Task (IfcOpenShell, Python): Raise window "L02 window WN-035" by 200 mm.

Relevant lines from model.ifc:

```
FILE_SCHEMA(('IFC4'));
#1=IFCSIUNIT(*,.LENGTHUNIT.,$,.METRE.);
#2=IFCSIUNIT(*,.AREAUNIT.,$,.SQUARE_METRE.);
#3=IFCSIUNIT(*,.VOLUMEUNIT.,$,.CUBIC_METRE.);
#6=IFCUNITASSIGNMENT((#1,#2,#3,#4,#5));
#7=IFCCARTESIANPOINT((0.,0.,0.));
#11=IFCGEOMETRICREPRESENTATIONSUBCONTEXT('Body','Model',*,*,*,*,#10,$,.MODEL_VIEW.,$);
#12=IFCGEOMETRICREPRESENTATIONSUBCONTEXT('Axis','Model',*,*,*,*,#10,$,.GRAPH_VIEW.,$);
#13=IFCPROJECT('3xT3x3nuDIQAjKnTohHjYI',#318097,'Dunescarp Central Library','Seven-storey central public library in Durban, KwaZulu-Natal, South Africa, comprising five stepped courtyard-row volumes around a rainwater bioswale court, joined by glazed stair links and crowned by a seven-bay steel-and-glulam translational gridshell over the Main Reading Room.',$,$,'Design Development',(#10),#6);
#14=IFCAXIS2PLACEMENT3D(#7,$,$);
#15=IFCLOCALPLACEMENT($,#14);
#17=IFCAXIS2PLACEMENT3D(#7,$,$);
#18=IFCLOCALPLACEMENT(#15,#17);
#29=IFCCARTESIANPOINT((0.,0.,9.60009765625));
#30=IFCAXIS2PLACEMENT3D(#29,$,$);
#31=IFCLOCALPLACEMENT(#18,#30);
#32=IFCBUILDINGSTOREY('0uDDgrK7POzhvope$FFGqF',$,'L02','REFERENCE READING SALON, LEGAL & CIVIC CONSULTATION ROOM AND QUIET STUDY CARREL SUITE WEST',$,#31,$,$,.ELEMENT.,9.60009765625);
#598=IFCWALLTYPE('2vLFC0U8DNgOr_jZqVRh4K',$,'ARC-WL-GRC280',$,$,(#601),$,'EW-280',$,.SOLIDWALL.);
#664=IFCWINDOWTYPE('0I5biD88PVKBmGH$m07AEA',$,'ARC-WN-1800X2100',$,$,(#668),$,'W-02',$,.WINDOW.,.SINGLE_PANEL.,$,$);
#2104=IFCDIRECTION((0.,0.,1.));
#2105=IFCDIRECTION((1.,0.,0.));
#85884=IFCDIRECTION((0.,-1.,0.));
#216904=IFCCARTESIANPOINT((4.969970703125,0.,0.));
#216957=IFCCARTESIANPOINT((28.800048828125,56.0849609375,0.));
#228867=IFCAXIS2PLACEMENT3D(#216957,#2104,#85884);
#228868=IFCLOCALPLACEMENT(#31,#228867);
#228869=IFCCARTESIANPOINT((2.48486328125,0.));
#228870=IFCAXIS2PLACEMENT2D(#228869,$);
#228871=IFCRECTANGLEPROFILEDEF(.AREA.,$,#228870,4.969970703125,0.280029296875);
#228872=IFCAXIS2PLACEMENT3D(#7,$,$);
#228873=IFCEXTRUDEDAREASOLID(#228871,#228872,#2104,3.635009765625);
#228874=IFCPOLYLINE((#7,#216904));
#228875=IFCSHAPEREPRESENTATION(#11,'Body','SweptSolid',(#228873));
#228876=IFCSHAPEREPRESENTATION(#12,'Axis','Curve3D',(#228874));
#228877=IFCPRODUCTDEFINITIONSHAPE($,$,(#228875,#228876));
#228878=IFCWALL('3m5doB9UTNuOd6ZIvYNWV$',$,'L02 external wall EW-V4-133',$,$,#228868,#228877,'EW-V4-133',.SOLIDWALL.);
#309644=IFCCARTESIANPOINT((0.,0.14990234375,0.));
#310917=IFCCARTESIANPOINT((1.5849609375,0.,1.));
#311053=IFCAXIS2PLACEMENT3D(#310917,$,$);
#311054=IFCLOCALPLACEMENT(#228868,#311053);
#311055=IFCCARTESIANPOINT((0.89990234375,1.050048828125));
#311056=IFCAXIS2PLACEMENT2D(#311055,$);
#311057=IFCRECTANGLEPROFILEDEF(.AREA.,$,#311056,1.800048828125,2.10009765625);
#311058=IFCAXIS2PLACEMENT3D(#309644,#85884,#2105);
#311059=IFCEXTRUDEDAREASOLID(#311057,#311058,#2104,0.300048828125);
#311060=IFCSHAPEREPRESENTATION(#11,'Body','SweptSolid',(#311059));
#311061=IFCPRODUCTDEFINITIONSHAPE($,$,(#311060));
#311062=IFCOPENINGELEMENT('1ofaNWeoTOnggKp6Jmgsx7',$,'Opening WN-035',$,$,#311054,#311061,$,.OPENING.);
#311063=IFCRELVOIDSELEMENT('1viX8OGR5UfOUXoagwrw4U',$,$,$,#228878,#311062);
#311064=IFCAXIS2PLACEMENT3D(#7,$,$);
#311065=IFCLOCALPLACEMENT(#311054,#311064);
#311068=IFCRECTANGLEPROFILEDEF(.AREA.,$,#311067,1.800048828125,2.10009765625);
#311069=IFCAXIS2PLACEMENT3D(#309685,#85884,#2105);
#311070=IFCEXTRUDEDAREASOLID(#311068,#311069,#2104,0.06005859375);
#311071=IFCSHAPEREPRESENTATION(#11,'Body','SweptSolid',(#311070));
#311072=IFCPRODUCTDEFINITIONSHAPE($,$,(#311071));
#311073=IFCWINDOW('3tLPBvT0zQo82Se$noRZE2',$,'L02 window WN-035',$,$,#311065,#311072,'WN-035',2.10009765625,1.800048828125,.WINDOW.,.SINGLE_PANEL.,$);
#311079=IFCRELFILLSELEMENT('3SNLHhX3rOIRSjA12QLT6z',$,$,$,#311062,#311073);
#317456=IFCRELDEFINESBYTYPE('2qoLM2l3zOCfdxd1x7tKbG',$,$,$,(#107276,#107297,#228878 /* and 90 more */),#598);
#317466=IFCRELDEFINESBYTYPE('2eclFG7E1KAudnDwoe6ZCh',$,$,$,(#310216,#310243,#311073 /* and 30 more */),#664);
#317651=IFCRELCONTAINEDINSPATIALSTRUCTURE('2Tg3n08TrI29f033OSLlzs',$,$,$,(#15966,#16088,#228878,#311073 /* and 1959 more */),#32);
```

```python
import numpy as np
import ifcopenshell
import ifcopenshell.api.geometry
import ifcopenshell.util.placement
import ifcopenshell.util.unit

model = ifcopenshell.open("model.ifc")
unit_scale = ifcopenshell.util.unit.calculate_unit_scale(model)

window = model.by_guid("3tLPBvT0zQo82Se$noRZE2")
opening = window.FillsVoids[0].RelatingOpeningElement
dz = 0.2

shift = np.array([0.0, 0.0, dz])
# The window is placed relative to its opening, so it follows when the opening moves.
matrix = ifcopenshell.util.placement.get_local_placement(opening.ObjectPlacement)
matrix[:3, 3] += shift
ifcopenshell.api.geometry.edit_object_placement(
    model, product=opening, matrix=matrix, is_si=False, should_transform_children=True
)

print(f"moved by {dz * unit_scale:+.3f} m")

model.write("model-out.ifc")
```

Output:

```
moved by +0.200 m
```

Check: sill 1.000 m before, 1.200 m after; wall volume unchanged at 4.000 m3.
